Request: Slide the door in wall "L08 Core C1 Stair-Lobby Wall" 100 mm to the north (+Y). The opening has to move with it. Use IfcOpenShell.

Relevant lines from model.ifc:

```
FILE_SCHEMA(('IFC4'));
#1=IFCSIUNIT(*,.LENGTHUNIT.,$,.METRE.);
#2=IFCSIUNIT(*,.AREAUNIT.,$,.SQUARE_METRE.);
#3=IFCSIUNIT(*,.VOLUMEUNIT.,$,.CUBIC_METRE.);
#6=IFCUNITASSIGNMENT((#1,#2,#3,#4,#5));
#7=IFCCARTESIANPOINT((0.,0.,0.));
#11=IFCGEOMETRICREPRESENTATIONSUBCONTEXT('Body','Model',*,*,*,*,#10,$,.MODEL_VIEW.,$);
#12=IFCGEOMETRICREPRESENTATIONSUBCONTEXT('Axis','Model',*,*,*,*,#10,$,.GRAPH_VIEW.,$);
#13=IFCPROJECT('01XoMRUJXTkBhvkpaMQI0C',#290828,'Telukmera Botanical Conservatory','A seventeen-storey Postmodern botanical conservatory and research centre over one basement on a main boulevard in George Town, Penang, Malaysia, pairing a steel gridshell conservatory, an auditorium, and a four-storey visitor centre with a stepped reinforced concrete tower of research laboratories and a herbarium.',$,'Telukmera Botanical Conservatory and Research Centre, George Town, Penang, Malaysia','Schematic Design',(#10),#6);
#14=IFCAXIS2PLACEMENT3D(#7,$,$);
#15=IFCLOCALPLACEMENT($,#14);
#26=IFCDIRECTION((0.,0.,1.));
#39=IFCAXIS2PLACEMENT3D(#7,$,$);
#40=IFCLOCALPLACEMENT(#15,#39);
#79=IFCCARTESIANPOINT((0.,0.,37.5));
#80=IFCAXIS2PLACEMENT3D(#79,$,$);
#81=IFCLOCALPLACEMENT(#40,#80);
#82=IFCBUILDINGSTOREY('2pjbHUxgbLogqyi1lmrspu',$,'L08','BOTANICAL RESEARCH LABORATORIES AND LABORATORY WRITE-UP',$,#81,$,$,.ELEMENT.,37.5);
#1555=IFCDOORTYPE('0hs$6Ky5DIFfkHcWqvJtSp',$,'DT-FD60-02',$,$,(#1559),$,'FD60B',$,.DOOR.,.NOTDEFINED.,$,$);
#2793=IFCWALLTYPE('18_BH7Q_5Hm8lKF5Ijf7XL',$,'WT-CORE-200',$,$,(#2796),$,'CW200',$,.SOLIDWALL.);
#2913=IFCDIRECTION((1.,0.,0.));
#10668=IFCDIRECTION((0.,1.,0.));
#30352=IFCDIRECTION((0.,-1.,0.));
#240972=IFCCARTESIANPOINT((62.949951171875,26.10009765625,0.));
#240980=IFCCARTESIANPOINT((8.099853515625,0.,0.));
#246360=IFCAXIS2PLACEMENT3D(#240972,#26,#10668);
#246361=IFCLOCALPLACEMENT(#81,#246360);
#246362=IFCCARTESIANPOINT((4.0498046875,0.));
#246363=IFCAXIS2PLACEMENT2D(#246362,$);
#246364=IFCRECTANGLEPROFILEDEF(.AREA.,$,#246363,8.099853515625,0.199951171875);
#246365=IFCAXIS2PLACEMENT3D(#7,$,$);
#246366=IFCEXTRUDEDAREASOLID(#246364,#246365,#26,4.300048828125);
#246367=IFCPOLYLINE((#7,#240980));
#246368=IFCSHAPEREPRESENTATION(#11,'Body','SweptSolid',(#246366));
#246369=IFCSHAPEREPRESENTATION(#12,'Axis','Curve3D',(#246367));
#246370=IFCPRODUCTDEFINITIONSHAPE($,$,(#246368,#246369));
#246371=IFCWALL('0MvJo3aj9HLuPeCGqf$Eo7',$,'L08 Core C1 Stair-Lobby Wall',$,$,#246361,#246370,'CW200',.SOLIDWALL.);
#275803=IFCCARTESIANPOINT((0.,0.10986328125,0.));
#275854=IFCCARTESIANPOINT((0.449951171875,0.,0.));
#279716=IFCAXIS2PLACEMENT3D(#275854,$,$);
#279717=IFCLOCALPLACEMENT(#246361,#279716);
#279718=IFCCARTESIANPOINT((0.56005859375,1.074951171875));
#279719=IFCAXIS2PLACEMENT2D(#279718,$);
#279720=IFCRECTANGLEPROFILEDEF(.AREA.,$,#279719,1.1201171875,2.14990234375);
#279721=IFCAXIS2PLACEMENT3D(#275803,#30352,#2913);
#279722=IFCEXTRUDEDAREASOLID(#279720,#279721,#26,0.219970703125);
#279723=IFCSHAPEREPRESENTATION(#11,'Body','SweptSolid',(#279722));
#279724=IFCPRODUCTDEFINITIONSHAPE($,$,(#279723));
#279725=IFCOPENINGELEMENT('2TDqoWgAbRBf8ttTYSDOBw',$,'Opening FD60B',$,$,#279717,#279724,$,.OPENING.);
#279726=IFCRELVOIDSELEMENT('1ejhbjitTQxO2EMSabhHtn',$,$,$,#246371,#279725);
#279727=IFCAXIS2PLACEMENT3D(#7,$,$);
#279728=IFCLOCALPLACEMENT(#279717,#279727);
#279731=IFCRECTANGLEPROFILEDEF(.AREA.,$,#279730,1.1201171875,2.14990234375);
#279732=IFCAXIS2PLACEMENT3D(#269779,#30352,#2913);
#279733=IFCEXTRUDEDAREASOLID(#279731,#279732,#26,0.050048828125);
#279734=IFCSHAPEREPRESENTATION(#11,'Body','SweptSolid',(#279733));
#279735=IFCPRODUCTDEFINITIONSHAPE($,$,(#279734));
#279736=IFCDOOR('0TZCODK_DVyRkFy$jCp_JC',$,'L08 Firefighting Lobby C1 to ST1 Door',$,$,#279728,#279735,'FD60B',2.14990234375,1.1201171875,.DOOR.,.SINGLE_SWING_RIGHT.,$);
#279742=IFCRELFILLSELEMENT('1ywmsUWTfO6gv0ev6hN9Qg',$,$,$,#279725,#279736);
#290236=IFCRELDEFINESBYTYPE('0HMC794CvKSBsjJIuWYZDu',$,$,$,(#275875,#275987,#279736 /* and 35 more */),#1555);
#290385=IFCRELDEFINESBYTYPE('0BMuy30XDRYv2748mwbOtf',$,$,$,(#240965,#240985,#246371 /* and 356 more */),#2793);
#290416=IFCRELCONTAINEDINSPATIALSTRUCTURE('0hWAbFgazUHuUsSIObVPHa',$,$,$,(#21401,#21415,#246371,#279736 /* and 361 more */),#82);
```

```python
import ifcopenshell
import ifcopenshell.api.geometry
import ifcopenshell.util.placement
import ifcopenshell.util.unit

model = ifcopenshell.open("model.ifc")
unit_scale = ifcopenshell.util.unit.calculate_unit_scale(model)

door = model.by_guid("0TZCODK_DVyRkFy$jCp_JC")
opening = door.FillsVoids[0].RelatingOpeningElement
wall = opening.VoidsElements[0].RelatingBuildingElement

wall_matrix = ifcopenshell.util.placement.get_local_placement(wall.ObjectPlacement)
shift = wall_matrix[:3, 0] * 0.1 / unit_scale
before = ifcopenshell.util.placement.get_local_placement(door.ObjectPlacement)[:3, 3].copy()

# The door is placed relative to its opening, so it follows when the opening moves.
matrix = ifcopenshell.util.placement.get_local_placement(opening.ObjectPlacement)
matrix[:3, 3] += shift
ifcopenshell.api.geometry.edit_object_placement(
    model, product=opening, matrix=matrix, is_si=False, should_transform_children=True
)

after = ifcopenshell.util.placement.get_local_placement(door.ObjectPlacement)[:3, 3]
print("door moved by", (after - before).round(3) + 0.0)

model.write("model-out.ifc")
```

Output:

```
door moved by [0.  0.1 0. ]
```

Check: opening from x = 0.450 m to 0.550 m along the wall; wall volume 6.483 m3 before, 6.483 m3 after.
